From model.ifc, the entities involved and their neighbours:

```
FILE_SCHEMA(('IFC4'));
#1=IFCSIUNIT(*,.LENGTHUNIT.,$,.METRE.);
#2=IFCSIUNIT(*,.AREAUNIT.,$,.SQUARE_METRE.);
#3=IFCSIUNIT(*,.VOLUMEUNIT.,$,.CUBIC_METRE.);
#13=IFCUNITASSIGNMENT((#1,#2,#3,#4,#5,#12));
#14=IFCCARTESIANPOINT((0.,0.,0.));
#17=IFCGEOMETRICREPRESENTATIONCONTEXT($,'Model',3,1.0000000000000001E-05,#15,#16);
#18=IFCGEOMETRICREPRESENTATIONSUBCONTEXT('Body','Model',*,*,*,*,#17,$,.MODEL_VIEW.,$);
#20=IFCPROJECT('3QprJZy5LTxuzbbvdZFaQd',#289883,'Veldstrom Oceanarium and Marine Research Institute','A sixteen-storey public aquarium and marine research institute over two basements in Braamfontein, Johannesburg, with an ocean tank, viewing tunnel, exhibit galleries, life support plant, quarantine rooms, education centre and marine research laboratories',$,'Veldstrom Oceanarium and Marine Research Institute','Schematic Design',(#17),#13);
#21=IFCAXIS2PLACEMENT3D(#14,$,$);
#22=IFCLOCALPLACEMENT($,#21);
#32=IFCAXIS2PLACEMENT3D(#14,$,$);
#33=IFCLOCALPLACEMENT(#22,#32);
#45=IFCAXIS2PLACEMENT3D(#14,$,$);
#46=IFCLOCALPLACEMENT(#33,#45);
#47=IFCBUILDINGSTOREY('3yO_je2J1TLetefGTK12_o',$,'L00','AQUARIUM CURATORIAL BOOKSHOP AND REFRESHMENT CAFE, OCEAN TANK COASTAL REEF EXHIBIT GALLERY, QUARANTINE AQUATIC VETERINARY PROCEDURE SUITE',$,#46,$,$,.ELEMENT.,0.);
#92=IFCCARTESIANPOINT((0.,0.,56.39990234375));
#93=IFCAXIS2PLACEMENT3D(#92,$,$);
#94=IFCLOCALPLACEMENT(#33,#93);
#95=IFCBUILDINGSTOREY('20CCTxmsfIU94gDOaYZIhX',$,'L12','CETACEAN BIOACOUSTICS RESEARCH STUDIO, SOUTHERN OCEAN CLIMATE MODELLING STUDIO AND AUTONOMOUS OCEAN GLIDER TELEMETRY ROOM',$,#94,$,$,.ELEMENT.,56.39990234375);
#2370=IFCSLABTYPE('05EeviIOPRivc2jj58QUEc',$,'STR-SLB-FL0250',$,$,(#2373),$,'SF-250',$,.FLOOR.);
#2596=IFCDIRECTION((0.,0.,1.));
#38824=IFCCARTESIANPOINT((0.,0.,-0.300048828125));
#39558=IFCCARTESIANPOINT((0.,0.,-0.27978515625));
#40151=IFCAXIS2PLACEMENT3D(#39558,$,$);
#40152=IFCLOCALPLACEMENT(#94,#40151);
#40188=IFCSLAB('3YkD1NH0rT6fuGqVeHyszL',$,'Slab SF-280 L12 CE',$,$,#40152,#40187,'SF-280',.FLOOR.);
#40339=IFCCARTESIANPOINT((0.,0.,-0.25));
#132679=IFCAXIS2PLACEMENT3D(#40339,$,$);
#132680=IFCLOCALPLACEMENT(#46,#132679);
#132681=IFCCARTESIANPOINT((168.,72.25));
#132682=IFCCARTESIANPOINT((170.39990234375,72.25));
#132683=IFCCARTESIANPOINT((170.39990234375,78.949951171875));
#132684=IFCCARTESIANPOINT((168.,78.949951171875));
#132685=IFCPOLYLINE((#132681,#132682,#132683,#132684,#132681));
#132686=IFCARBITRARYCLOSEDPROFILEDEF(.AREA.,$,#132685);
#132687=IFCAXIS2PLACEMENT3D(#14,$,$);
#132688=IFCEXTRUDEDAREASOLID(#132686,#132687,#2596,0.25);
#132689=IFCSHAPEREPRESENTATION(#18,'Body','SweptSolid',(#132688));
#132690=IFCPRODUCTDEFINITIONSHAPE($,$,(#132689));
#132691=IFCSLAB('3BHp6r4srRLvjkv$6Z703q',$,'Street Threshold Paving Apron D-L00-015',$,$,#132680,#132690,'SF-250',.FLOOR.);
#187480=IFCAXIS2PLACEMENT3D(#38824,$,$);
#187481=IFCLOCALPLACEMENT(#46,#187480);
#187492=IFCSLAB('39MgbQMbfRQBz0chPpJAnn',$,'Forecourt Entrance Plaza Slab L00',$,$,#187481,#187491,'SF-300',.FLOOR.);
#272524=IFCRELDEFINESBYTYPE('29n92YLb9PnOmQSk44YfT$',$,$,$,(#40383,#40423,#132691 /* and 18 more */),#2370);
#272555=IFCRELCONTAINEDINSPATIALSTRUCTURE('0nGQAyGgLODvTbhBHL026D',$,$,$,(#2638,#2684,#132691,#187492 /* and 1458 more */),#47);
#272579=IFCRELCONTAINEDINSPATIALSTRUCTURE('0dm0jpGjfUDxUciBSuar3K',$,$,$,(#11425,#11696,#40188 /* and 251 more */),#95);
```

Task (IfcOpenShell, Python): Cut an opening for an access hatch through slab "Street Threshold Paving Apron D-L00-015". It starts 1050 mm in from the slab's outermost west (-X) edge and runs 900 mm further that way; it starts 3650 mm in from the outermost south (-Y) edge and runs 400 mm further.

```python
import numpy as np
import ifcopenshell
import ifcopenshell.api.feature
import ifcopenshell.api.geometry
import ifcopenshell.api.root
import ifcopenshell.geom
import ifcopenshell.util.placement
import ifcopenshell.util.representation
import ifcopenshell.util.shape
import ifcopenshell.util.unit

model = ifcopenshell.open("model.ifc")
unit_scale = ifcopenshell.util.unit.calculate_unit_scale(model)
settings = ifcopenshell.geom.settings()


def volume(element):
    """Net volume in cubic metres, openings subtracted."""
    shape = ifcopenshell.geom.create_shape(settings, element)
    return ifcopenshell.util.shape.get_volume(shape.geometry)


slab = model.by_guid("3BHp6r4srRLvjkv$6Z703q")
before = volume(slab)

# Extent in the slab's own axes, in metres. The edges named are its -X and -Y sides.
slab_shape = ifcopenshell.geom.create_shape(settings, slab)
vertices = ifcopenshell.util.shape.get_vertices(slab_shape.geometry)
x_min, y_min, bottom = vertices.min(axis=0)
top = vertices[:, 2].max()

opening = ifcopenshell.api.root.create_entity(model, ifc_class="IfcOpeningElement", name="Access hatch opening", predefined_type="OPENING")
context = ifcopenshell.util.representation.get_context(model, "Model", "Body", "MODEL_VIEW")
width, depth = 0.9, 0.4
outline = [(0.0, 0.0), (width, 0.0), (width, depth), (0.0, depth), (0.0, 0.0)]
# Overshoot both faces by 50 mm so the cut is clean.
shape = ifcopenshell.api.geometry.add_slab_representation(
    model, context=context, depth=top - bottom + 0.1, polyline=outline
)
ifcopenshell.api.geometry.assign_representation(model, product=opening, representation=shape)

matrix = ifcopenshell.util.placement.get_local_placement(slab.ObjectPlacement)
matrix[:, 3] = matrix @ np.append(np.array([x_min + 1.05, y_min + 3.65, bottom - 0.05]) / unit_scale, 1.0)
ifcopenshell.api.geometry.edit_object_placement(model, product=opening, matrix=matrix, is_si=False)
ifcopenshell.api.feature.add_feature(model, feature=opening, element=slab)

after = volume(slab)

print(f"slab volume {before:.3f} -> {after:.3f} m3")

model.write("model_updated.ifc")
```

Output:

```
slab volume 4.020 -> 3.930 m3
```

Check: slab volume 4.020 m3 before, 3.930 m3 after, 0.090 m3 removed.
